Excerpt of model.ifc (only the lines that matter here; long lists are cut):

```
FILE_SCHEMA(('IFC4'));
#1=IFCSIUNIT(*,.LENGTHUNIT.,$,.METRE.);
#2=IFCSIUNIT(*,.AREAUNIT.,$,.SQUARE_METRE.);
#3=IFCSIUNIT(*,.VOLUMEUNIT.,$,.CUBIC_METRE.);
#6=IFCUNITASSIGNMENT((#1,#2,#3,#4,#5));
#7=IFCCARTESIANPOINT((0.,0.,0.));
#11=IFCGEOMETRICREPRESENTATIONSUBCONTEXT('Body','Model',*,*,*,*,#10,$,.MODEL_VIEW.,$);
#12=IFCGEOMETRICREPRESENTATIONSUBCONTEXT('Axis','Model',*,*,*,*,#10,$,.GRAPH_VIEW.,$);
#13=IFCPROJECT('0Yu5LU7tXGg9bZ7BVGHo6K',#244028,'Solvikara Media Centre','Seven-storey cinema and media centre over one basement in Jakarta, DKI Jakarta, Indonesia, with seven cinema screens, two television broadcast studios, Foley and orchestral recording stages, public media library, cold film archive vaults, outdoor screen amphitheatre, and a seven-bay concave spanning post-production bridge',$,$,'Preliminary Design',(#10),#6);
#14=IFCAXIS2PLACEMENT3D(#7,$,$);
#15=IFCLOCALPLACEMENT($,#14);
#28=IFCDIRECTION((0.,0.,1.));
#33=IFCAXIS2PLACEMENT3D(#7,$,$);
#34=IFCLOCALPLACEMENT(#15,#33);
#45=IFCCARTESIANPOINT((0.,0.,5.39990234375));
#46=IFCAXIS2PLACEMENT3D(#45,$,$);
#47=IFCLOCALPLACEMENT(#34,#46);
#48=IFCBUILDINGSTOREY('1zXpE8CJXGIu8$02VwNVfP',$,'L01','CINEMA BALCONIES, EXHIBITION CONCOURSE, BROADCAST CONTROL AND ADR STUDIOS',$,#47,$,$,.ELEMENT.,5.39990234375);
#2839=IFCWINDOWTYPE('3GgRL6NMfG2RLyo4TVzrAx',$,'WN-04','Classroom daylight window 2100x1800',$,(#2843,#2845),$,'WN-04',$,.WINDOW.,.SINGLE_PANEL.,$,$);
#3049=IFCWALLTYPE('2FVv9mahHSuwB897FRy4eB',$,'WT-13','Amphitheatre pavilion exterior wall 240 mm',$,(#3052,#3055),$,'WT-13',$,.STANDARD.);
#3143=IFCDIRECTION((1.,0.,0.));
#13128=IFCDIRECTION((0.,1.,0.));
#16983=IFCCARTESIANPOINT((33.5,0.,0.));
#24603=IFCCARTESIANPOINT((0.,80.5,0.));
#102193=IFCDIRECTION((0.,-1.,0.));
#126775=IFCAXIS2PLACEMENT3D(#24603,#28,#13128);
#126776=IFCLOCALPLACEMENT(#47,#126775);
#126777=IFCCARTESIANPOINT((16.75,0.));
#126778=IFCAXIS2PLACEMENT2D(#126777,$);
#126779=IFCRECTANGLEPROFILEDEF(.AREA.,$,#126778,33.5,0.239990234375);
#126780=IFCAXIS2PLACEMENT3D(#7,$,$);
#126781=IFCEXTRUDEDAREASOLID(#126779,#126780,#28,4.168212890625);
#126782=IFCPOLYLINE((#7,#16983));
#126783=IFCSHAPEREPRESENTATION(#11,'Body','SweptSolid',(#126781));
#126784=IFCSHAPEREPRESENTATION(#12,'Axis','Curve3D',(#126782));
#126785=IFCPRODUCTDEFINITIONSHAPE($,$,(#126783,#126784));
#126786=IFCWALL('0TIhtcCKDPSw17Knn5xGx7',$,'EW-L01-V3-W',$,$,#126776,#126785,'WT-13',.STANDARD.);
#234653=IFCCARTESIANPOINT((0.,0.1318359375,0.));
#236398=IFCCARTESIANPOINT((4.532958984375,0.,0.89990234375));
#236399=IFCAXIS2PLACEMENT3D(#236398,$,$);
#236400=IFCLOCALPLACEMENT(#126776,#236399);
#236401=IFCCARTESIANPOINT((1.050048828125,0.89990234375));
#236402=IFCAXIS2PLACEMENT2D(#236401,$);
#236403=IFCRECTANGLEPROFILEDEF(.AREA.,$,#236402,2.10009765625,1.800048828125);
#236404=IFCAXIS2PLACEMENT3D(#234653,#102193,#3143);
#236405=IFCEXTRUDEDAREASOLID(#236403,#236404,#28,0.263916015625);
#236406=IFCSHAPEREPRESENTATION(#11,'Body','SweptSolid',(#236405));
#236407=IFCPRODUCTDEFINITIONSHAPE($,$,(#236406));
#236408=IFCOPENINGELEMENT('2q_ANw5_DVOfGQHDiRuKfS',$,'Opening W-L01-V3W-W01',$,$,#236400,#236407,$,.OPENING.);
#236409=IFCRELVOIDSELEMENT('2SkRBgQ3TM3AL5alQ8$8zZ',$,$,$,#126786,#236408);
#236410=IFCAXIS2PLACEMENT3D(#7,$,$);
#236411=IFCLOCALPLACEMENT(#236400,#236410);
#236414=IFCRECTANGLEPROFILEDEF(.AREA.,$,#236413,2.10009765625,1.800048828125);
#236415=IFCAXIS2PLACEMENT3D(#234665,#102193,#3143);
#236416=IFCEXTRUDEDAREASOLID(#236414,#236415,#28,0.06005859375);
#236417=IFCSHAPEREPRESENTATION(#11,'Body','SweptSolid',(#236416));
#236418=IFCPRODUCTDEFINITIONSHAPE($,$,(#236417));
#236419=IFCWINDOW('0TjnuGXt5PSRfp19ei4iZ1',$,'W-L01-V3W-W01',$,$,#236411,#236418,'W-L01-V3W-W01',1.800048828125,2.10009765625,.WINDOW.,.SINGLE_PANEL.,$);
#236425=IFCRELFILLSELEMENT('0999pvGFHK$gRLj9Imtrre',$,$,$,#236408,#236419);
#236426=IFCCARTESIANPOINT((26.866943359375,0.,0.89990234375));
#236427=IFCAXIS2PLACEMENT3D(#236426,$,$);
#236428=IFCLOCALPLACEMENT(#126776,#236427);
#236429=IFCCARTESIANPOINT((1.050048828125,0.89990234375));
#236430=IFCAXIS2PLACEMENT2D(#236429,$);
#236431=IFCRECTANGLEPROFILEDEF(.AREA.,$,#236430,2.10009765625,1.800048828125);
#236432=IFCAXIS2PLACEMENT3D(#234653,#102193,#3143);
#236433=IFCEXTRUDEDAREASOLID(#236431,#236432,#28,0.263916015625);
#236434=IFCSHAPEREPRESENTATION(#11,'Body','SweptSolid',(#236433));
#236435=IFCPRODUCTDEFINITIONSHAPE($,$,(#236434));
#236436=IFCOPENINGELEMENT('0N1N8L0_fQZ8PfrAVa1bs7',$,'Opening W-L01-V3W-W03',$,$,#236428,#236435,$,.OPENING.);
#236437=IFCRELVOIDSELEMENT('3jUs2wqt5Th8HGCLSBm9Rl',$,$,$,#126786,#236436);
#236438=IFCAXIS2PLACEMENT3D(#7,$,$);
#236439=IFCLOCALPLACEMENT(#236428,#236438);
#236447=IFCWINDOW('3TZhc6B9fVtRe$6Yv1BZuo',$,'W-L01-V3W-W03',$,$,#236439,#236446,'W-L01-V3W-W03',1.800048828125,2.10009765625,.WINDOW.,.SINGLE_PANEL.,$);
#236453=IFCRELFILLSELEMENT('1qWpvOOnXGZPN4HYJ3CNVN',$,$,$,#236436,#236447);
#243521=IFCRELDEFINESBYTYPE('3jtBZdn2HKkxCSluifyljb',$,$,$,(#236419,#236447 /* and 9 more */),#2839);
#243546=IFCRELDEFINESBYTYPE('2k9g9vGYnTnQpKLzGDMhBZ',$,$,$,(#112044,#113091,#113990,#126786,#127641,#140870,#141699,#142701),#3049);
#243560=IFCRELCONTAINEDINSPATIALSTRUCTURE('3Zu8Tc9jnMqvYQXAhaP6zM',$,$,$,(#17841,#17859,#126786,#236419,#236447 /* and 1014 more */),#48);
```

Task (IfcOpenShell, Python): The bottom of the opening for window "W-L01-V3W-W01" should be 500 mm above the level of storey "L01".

```python
import numpy as np
import ifcopenshell
import ifcopenshell.api.geometry
import ifcopenshell.geom
import ifcopenshell.util.element
import ifcopenshell.util.placement
import ifcopenshell.util.shape
import ifcopenshell.util.unit

model = ifcopenshell.open("model.ifc")
unit_scale = ifcopenshell.util.unit.calculate_unit_scale(model)

window = model.by_guid("0TjnuGXt5PSRfp19ei4iZ1")
opening = window.FillsVoids[0].RelatingOpeningElement
storey = ifcopenshell.util.element.get_container(window, ifc_class="IfcBuildingStorey")
level = ifcopenshell.util.placement.get_local_placement(storey.ObjectPlacement)[2, 3]

# The opening's origin need not be at the sill, so measure its lowest point.
shape = ifcopenshell.geom.create_shape(ifcopenshell.geom.settings(), opening)
bottom = ifcopenshell.util.shape.get_shape_bottom_elevation(shape, shape.geometry) / unit_scale
dz = level + 0.5 / unit_scale - bottom

shift = np.array([0.0, 0.0, dz])
# The window is placed relative to its opening, so it follows when the opening moves.
matrix = ifcopenshell.util.placement.get_local_placement(opening.ObjectPlacement)
matrix[:3, 3] += shift
ifcopenshell.api.geometry.edit_object_placement(
    model, product=opening, matrix=matrix, is_si=False, should_transform_children=True
)

print(f"moved by {dz * unit_scale:+.3f} m")

model.write("model_edited.ifc")
```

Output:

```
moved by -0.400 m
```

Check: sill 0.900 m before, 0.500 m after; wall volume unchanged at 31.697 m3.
